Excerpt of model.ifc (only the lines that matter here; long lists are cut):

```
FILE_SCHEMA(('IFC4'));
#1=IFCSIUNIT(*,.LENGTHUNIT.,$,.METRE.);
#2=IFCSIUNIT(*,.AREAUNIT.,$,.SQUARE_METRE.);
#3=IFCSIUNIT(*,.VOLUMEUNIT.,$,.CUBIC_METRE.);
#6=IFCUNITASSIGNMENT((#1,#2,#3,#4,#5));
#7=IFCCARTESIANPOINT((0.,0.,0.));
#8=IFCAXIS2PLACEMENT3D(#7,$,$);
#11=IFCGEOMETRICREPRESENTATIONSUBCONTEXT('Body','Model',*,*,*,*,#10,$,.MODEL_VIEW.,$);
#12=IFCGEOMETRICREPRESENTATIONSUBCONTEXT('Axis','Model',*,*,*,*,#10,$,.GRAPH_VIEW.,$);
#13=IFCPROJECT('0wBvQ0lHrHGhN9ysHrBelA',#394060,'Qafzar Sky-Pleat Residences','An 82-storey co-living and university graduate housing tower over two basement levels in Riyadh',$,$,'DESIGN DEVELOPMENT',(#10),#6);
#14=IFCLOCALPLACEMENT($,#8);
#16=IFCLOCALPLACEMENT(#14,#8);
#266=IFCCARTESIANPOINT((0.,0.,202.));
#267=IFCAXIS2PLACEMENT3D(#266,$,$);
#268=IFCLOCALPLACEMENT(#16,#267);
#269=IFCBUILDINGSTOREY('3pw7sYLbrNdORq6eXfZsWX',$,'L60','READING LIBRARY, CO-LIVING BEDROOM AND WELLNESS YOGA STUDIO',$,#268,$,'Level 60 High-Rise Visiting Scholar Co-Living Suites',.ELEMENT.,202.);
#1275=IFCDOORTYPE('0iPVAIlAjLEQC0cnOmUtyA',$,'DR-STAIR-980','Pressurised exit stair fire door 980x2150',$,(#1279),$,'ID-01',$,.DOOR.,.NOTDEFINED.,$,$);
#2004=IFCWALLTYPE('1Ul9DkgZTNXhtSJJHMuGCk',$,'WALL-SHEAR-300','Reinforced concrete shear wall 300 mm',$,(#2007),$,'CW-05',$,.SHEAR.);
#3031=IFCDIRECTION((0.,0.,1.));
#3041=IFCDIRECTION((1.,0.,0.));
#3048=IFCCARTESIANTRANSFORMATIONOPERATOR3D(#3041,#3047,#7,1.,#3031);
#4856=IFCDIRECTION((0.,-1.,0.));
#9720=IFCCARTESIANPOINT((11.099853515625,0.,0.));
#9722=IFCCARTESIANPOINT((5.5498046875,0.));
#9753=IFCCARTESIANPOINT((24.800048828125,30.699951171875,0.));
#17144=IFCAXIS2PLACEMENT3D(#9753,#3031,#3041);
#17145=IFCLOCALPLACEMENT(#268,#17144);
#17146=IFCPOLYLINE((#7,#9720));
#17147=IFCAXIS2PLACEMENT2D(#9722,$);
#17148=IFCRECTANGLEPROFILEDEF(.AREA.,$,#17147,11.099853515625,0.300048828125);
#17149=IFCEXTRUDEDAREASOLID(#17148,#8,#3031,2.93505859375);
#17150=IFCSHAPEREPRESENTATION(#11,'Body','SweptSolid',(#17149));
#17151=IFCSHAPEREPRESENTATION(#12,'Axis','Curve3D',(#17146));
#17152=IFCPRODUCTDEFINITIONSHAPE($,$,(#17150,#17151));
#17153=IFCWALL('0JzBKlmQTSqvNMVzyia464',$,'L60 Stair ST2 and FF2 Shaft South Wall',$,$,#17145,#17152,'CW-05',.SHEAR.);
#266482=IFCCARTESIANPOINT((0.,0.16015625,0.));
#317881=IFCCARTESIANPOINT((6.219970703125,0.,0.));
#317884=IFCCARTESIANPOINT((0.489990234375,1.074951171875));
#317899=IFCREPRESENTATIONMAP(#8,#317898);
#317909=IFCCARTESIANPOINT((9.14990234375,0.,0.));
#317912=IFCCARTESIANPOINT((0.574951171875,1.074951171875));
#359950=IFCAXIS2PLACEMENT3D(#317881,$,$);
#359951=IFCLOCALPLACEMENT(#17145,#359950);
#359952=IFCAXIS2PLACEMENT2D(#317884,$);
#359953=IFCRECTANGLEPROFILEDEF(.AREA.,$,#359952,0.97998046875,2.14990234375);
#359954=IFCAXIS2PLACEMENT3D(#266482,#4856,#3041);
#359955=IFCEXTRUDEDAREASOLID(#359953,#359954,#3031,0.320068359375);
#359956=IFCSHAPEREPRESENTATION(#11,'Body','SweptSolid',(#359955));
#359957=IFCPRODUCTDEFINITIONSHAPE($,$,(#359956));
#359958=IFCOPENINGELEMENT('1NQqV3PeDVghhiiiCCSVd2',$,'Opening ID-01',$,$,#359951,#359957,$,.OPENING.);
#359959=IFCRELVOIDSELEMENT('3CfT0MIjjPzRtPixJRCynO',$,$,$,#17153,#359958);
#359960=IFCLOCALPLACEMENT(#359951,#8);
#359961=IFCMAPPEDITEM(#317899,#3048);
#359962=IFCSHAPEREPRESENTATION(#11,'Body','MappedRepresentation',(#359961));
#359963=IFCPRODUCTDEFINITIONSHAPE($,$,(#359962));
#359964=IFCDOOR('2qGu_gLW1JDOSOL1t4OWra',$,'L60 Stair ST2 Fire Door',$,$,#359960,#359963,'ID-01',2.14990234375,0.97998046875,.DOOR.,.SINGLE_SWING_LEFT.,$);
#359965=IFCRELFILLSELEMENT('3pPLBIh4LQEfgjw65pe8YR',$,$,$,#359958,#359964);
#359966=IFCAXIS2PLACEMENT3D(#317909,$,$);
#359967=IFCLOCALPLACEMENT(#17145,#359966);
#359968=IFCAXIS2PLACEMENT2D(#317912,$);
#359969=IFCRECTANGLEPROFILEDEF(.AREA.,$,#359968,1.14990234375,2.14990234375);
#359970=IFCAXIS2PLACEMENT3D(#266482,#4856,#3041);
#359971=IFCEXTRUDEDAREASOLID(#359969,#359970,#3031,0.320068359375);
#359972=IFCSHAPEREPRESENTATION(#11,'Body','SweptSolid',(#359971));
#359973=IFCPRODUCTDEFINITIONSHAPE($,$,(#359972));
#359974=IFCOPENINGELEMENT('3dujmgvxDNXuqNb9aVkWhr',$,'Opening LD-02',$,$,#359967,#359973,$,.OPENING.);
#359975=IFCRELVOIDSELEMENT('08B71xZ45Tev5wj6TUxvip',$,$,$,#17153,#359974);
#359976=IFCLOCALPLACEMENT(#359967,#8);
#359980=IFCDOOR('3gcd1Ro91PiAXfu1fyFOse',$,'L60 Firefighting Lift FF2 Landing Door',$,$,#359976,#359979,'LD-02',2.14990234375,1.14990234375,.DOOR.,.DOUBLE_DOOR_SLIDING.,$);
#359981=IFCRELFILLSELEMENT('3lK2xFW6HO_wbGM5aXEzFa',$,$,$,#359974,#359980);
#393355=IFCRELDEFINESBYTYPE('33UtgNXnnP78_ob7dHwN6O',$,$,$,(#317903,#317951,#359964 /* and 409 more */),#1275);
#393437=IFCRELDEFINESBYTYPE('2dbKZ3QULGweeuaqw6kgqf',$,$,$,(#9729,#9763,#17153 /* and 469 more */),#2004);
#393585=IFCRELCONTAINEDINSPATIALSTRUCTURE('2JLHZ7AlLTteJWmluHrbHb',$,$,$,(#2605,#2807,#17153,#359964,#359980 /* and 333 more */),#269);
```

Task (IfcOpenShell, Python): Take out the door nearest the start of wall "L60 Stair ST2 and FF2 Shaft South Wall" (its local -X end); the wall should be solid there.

```python
import ifcopenshell
import ifcopenshell.api.feature
import ifcopenshell.api.root
import ifcopenshell.geom
import ifcopenshell.util.shape

model = ifcopenshell.open("model.ifc")
settings = ifcopenshell.geom.settings()


def volume(element):
    """Net volume in cubic metres, openings subtracted."""
    shape = ifcopenshell.geom.create_shape(settings, element)
    return ifcopenshell.util.shape.get_volume(shape.geometry)


door = model.by_guid("2qGu_gLW1JDOSOL1t4OWra")
opening = door.FillsVoids[0].RelatingOpeningElement
wall = opening.VoidsElements[0].RelatingBuildingElement
before = volume(wall)

ifcopenshell.api.root.remove_product(model, product=door)
ifcopenshell.api.feature.remove_feature(model, feature=opening)

after = volume(wall)

print(f"wall volume {before:.3f} -> {after:.3f} m3")

model.write("model_rev.ifc")
```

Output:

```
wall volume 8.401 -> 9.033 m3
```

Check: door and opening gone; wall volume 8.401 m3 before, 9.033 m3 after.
